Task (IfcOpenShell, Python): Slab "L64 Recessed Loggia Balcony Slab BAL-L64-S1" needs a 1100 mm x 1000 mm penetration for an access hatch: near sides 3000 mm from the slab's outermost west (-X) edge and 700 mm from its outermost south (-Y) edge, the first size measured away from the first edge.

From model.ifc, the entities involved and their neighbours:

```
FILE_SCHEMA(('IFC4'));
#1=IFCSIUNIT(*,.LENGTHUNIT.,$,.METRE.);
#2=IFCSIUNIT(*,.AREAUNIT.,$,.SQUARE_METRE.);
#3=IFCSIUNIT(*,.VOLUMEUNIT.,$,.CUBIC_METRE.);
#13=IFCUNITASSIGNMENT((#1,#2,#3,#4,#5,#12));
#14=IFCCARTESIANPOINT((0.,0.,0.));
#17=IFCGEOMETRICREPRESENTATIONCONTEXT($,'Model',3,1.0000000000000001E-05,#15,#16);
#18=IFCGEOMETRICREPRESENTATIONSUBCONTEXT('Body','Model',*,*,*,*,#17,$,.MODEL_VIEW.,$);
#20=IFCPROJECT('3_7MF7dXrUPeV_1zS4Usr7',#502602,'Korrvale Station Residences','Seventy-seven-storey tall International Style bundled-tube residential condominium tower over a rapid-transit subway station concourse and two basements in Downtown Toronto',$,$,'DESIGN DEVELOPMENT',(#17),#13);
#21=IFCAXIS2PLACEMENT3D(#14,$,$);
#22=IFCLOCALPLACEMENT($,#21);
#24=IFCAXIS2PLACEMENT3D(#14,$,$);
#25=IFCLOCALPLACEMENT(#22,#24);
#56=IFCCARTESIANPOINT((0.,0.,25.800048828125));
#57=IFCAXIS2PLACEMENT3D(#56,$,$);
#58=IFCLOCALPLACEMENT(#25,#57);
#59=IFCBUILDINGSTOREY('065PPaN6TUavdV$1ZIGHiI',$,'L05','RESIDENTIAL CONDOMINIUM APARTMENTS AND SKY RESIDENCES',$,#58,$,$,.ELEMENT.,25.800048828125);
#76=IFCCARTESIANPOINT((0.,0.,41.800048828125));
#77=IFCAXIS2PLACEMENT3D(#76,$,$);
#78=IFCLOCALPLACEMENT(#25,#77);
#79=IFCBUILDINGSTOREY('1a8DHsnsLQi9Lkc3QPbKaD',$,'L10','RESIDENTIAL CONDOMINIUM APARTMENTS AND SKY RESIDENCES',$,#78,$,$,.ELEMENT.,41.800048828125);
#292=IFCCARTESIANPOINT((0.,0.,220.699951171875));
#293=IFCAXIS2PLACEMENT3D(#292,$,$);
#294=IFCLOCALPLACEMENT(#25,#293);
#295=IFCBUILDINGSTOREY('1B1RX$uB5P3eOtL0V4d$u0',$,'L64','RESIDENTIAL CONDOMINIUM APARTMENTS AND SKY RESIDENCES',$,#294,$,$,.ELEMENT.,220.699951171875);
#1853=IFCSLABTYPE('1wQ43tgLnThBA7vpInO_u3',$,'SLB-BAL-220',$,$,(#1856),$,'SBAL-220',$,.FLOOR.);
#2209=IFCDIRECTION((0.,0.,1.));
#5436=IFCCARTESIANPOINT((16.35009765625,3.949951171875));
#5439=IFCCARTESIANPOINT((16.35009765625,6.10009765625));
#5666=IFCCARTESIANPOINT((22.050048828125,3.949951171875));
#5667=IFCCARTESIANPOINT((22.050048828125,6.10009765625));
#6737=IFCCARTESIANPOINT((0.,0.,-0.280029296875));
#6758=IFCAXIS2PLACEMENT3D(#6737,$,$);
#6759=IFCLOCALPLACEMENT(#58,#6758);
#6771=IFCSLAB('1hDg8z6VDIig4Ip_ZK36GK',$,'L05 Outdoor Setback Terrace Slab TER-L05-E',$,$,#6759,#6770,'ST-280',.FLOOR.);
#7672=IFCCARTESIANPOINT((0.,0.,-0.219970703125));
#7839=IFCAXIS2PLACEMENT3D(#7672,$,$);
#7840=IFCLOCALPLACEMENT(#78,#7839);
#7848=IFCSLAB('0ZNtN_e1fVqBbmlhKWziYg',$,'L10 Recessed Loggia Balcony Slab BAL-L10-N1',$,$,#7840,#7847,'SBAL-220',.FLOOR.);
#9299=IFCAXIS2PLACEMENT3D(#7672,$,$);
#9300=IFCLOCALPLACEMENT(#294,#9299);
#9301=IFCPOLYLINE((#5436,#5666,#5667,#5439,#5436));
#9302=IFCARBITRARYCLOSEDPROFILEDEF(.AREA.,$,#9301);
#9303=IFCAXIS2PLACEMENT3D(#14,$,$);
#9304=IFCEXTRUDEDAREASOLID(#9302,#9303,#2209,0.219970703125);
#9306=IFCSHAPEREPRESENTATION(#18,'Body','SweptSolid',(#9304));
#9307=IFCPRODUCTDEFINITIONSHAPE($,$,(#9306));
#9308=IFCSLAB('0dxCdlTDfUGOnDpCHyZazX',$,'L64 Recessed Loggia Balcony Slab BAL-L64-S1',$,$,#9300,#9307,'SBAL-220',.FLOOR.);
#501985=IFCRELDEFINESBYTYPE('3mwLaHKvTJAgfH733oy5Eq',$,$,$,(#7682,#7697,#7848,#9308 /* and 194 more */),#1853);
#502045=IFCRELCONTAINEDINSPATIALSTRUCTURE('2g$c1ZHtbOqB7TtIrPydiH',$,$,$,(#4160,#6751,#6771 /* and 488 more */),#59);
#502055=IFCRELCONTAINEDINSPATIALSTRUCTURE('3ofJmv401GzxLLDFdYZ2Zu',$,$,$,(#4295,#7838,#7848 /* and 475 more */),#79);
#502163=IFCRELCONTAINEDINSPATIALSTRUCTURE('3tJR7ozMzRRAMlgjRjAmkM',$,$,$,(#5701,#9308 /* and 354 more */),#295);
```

```python
import numpy as np
import ifcopenshell
import ifcopenshell.api.feature
import ifcopenshell.api.geometry
import ifcopenshell.api.root
import ifcopenshell.geom
import ifcopenshell.util.placement
import ifcopenshell.util.representation
import ifcopenshell.util.shape
import ifcopenshell.util.unit

model = ifcopenshell.open("model.ifc")
unit_scale = ifcopenshell.util.unit.calculate_unit_scale(model)
settings = ifcopenshell.geom.settings()


def volume(element):
    """Net volume in cubic metres, openings subtracted."""
    shape = ifcopenshell.geom.create_shape(settings, element)
    return ifcopenshell.util.shape.get_volume(shape.geometry)


slab = model.by_guid("0dxCdlTDfUGOnDpCHyZazX")
before = volume(slab)

# Extent in the slab's own axes, in metres. The edges named are its -X and -Y sides.
slab_shape = ifcopenshell.geom.create_shape(settings, slab)
vertices = ifcopenshell.util.shape.get_vertices(slab_shape.geometry)
x_min, y_min, bottom = vertices.min(axis=0)
top = vertices[:, 2].max()

opening = ifcopenshell.api.root.create_entity(model, ifc_class="IfcOpeningElement", name="Access hatch opening", predefined_type="OPENING")
context = ifcopenshell.util.representation.get_context(model, "Model", "Body", "MODEL_VIEW")
width, depth = 1.1, 1
outline = [(0.0, 0.0), (width, 0.0), (width, depth), (0.0, depth), (0.0, 0.0)]
# Overshoot both faces by 50 mm so the cut is clean.
shape = ifcopenshell.api.geometry.add_slab_representation(
    model, context=context, depth=top - bottom + 0.1, polyline=outline
)
ifcopenshell.api.geometry.assign_representation(model, product=opening, representation=shape)

matrix = ifcopenshell.util.placement.get_local_placement(slab.ObjectPlacement)
matrix[:, 3] = matrix @ np.append(np.array([x_min + 3, y_min + 0.7, bottom - 0.05]) / unit_scale, 1.0)
ifcopenshell.api.geometry.edit_object_placement(model, product=opening, matrix=matrix, is_si=False)
ifcopenshell.api.feature.add_feature(model, feature=opening, element=slab)

after = volume(slab)

print(f"slab volume {before:.3f} -> {after:.3f} m3")

model.write("model_v2.ifc")
```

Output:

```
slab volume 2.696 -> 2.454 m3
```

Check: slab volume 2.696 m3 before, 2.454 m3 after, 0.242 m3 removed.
